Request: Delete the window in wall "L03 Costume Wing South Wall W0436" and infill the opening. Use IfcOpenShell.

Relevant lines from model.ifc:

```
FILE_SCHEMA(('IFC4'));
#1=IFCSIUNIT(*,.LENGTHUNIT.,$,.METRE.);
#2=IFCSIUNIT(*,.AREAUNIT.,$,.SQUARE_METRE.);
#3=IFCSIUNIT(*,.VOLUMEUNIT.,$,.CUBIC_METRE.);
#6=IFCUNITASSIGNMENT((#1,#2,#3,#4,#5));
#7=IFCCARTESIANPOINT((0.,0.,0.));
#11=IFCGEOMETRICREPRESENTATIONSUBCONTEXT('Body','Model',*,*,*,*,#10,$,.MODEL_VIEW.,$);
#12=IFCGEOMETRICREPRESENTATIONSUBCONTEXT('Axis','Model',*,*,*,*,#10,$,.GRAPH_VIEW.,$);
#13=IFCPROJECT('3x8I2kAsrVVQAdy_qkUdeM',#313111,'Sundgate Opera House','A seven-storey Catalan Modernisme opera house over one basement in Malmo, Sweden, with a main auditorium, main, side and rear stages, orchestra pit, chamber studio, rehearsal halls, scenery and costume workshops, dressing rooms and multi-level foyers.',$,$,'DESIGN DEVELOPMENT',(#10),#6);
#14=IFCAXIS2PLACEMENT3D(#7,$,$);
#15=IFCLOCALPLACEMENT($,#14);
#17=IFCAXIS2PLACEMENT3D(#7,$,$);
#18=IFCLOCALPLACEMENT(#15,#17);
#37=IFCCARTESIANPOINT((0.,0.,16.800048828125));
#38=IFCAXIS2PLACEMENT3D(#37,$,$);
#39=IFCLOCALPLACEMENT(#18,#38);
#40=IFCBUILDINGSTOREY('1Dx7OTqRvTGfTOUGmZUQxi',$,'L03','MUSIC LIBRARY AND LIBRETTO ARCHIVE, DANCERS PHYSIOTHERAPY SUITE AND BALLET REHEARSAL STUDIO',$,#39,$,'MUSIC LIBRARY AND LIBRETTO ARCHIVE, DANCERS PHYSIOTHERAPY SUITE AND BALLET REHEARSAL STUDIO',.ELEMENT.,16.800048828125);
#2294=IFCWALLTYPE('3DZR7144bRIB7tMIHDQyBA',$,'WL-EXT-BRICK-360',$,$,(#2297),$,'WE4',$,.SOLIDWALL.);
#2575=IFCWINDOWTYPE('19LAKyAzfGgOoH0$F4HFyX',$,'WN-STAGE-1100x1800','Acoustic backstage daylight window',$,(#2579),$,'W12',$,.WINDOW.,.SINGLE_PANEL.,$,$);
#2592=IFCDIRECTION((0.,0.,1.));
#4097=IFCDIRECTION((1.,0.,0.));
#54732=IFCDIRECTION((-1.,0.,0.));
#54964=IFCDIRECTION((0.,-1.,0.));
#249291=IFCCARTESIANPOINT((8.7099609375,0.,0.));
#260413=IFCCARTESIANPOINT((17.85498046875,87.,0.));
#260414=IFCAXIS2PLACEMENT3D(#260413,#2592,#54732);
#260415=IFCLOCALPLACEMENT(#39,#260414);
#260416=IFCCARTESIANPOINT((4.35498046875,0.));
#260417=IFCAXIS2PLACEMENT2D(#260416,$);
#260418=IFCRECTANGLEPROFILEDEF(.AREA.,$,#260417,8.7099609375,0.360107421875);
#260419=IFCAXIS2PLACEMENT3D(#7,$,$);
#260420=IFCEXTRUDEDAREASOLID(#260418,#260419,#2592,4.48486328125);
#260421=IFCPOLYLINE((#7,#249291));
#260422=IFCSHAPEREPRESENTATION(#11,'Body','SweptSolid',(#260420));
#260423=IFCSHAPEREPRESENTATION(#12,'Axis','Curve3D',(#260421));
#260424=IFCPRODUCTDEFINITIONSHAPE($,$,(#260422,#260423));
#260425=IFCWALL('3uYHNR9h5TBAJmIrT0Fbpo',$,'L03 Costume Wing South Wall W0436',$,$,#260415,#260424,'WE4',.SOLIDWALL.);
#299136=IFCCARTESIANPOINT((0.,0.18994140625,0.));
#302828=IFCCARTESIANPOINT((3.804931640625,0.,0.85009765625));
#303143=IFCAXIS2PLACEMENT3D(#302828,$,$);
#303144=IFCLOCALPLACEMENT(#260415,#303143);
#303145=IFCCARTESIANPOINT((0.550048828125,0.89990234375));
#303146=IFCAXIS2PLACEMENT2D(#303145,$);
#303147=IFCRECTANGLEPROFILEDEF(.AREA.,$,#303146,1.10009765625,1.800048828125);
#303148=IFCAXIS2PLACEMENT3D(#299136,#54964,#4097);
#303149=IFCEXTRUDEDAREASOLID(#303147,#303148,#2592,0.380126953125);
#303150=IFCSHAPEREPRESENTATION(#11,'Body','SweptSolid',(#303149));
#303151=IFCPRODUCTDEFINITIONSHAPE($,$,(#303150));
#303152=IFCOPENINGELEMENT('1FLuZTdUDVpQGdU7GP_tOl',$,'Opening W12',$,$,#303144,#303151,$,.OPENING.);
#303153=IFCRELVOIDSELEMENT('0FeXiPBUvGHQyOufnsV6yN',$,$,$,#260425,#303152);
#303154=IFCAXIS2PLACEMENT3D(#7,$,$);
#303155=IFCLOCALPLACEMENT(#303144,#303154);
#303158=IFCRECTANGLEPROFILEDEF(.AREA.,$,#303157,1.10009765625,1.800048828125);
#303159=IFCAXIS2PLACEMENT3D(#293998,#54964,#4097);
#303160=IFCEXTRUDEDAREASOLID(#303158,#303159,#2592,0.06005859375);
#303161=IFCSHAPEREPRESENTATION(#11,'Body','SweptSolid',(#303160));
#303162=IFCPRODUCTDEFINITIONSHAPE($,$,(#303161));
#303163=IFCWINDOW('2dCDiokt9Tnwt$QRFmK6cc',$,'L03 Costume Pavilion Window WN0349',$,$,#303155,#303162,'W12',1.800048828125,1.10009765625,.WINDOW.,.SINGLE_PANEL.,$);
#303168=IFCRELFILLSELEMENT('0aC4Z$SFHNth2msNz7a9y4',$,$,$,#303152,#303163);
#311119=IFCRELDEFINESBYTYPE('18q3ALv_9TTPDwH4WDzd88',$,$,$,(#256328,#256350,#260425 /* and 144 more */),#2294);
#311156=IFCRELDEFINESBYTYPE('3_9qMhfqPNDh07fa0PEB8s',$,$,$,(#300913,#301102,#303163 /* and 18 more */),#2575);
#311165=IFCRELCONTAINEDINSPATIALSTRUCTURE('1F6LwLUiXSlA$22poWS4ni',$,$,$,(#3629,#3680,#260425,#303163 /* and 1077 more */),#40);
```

```python
import ifcopenshell
import ifcopenshell.api.feature
import ifcopenshell.api.root
import ifcopenshell.geom
import ifcopenshell.util.shape

model = ifcopenshell.open("model.ifc")
settings = ifcopenshell.geom.settings()


def volume(element):
    """Net volume in cubic metres, openings subtracted."""
    shape = ifcopenshell.geom.create_shape(settings, element)
    return ifcopenshell.util.shape.get_volume(shape.geometry)


window = model.by_id(303163)
opening = window.FillsVoids[0].RelatingOpeningElement
wall = opening.VoidsElements[0].RelatingBuildingElement
before = volume(wall)

ifcopenshell.api.root.remove_product(model, product=window)
ifcopenshell.api.feature.remove_feature(model, feature=opening)

after = volume(wall)

print(f"wall volume {before:.3f} -> {after:.3f} m3")

model.write("model_v2.ifc")
```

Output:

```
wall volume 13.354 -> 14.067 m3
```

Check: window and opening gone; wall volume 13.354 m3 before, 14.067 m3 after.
